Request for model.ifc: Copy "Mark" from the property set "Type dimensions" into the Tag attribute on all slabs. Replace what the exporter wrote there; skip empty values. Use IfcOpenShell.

First a look at what the model holds.

```python
import ifcopenshell
import ifcopenshell.util.element

model = ifcopenshell.open("model.ifc")
print(model.schema)
slabs = model.by_type("IfcSlab")
print(len(slabs), "slabs")
for e in slabs[:8]:
    source = ifcopenshell.util.element.get_pset(e, "Type dimensions", "Mark")
    target = e.Tag
    print(e.id(), repr(source), repr(target), sep=" | ")
```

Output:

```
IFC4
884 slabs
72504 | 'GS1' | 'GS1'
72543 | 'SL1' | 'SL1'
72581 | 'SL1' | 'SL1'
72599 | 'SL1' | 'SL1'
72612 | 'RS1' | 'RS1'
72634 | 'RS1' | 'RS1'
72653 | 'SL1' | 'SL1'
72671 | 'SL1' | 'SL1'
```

```python
import ifcopenshell
import ifcopenshell.util.element

model = ifcopenshell.open("model.ifc")

count = 0
for e in model.by_type("IfcSlab"):
    value = ifcopenshell.util.element.get_pset(e, "Type dimensions", "Mark")
    current = e.Tag
    if not value or not value.strip() or current == value:
        continue
    e.Tag = value
    count += 1

print(count, "slabs updated")

model.write("model_edited.ifc")
```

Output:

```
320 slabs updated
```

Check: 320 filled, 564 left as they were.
